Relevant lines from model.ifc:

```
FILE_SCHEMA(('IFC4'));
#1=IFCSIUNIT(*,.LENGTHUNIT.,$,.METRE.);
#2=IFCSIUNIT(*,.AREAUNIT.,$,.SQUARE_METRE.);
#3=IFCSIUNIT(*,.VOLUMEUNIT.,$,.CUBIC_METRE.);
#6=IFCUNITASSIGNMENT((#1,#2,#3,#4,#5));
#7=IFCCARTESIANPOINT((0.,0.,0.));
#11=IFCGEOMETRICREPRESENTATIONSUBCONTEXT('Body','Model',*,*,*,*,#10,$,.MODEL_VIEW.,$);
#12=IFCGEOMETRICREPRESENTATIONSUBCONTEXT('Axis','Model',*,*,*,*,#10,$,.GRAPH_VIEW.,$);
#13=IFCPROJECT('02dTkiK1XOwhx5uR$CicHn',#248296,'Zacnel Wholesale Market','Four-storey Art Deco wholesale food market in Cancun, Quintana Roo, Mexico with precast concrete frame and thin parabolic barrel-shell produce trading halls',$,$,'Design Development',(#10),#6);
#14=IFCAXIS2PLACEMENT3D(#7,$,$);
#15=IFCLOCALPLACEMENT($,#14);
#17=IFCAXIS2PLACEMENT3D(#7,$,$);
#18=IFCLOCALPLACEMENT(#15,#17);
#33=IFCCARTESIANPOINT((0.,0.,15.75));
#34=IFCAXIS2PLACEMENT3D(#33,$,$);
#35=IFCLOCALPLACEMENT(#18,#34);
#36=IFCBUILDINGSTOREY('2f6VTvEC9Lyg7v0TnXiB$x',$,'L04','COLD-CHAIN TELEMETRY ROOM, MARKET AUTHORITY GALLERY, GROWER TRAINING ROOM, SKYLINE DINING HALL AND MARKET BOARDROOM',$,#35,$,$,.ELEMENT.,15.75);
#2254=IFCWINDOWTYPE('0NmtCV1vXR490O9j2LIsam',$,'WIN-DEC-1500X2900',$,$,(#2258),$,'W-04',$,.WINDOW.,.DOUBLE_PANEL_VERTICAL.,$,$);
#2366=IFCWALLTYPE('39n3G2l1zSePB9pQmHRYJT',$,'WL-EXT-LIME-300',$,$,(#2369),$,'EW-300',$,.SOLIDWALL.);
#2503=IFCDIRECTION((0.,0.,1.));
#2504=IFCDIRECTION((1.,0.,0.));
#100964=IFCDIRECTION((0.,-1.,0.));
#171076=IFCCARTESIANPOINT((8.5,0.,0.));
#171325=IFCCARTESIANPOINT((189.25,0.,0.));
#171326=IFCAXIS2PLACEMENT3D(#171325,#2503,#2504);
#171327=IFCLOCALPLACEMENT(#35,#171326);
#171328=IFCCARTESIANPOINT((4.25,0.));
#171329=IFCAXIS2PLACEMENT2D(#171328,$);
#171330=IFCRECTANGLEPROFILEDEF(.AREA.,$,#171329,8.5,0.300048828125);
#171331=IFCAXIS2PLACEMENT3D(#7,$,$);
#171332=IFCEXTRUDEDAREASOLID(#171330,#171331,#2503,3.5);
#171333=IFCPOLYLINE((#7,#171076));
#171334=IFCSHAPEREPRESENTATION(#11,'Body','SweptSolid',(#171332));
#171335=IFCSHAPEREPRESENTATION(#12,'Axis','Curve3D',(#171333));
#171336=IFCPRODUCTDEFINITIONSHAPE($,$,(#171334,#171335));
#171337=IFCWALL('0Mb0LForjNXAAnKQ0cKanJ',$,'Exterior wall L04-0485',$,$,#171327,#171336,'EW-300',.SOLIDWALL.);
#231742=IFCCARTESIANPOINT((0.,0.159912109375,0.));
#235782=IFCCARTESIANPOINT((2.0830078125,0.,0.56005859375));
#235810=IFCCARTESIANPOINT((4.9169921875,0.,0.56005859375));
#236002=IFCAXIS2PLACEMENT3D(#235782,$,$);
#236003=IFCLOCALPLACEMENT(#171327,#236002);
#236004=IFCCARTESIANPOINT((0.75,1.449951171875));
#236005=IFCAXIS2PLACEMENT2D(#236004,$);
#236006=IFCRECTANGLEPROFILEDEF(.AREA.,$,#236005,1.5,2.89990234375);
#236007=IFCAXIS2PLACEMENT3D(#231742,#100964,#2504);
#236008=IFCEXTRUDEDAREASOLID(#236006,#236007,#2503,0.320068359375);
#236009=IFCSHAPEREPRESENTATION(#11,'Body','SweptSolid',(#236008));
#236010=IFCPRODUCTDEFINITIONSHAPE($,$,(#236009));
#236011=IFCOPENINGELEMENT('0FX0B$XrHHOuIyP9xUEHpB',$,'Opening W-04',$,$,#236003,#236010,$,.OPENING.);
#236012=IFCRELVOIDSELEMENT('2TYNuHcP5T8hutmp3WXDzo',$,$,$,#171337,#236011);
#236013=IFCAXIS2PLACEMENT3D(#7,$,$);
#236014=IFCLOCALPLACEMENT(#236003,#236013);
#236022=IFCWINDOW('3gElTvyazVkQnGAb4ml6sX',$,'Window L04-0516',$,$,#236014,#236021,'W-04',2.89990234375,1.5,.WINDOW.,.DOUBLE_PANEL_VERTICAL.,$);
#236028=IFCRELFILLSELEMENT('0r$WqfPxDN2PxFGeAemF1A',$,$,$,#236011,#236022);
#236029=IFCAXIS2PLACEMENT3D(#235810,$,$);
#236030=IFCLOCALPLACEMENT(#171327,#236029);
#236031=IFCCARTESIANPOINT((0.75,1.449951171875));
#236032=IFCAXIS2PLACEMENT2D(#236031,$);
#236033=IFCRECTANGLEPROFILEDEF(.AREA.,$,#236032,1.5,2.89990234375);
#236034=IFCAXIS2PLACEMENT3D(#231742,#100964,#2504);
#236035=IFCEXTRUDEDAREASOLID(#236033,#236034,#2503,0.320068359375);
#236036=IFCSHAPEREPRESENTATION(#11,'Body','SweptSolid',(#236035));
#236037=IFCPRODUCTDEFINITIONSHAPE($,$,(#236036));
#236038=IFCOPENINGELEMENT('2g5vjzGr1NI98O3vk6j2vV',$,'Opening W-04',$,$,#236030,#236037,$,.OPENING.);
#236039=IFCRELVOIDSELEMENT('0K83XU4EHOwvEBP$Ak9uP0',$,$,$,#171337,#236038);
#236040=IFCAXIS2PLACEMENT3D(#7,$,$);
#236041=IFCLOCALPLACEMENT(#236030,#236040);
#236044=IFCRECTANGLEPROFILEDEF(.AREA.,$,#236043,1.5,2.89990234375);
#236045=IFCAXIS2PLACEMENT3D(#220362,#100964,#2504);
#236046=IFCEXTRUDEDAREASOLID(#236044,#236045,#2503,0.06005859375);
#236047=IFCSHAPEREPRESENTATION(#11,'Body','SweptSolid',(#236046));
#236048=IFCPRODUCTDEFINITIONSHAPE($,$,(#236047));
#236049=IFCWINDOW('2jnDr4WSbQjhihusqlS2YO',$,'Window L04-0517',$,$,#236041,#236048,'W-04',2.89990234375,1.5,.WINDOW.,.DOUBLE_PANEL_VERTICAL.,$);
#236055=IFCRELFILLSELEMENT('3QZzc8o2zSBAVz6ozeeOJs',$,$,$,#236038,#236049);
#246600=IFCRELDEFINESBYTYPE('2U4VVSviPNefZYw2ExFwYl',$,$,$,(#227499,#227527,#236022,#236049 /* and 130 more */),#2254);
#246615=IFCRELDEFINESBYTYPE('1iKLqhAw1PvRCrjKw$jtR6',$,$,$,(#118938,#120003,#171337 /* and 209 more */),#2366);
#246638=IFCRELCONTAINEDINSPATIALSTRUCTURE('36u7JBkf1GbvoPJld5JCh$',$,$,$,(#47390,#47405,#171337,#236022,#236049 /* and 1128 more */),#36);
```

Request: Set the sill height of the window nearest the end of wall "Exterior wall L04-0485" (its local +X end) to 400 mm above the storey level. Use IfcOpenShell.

```python
import numpy as np
import ifcopenshell
import ifcopenshell.api.geometry
import ifcopenshell.geom
import ifcopenshell.util.element
import ifcopenshell.util.placement
import ifcopenshell.util.shape
import ifcopenshell.util.unit

model = ifcopenshell.open("model.ifc")
unit_scale = ifcopenshell.util.unit.calculate_unit_scale(model)

window = model.by_guid("2jnDr4WSbQjhihusqlS2YO")
opening = window.FillsVoids[0].RelatingOpeningElement
storey = ifcopenshell.util.element.get_container(window, ifc_class="IfcBuildingStorey")
level = ifcopenshell.util.placement.get_local_placement(storey.ObjectPlacement)[2, 3]

# The opening's origin need not be at the sill, so measure its lowest point.
shape = ifcopenshell.geom.create_shape(ifcopenshell.geom.settings(), opening)
bottom = ifcopenshell.util.shape.get_shape_bottom_elevation(shape, shape.geometry) / unit_scale
dz = level + 0.4 / unit_scale - bottom

shift = np.array([0.0, 0.0, dz])
# The window is placed relative to its opening, so it follows when the opening moves.
matrix = ifcopenshell.util.placement.get_local_placement(opening.ObjectPlacement)
matrix[:3, 3] += shift
ifcopenshell.api.geometry.edit_object_placement(
    model, product=opening, matrix=matrix, is_si=False, should_transform_children=True
)

print(f"moved by {dz * unit_scale:+.3f} m")

model.write("model_v2.ifc")
```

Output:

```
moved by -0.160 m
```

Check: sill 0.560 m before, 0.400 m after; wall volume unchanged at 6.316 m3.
